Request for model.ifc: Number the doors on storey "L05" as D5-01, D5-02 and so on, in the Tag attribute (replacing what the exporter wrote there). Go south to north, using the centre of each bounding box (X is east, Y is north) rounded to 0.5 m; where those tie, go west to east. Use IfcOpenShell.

First a look at what the model holds.

```python
import ifcopenshell
import ifcopenshell.util.element
import ifcopenshell.util.placement

model = ifcopenshell.open("model.ifc")
print(model.schema)
storey = next(s for s in model.by_type("IfcBuildingStorey") if s.Name == "L05")
doors = [e for e in ifcopenshell.util.element.get_decomposition(storey) if e.is_a("IfcDoor")]
for e in sorted(doors, key=lambda e: e.id()):
    origin = ifcopenshell.util.placement.get_local_placement(e.ObjectPlacement)[:3, 3]
    print(e.id(), e.Tag, e.Name, origin.round(2) + 0.0, sep=" | ")
```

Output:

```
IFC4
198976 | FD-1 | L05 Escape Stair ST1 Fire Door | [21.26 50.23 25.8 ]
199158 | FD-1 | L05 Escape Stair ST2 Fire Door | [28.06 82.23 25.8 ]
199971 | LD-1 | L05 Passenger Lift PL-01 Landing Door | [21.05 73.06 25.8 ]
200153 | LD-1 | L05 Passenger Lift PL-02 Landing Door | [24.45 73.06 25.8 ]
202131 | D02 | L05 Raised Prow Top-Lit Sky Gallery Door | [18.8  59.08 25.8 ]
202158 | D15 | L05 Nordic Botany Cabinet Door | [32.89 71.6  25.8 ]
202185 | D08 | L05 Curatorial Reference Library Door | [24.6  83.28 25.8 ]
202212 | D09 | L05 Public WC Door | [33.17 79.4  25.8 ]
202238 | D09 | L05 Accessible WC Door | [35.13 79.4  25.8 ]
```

```python
import ifcopenshell
import ifcopenshell.geom
import ifcopenshell.util.element
import ifcopenshell.util.shape

model = ifcopenshell.open("model.ifc")
settings = ifcopenshell.geom.settings()
settings.set("use-world-coords", True)


def centre(element):
    shape = ifcopenshell.geom.create_shape(settings, element)
    return ifcopenshell.util.shape.get_bbox_centroid(shape.geometry)


storey = next(s for s in model.by_type("IfcBuildingStorey") if s.Name == "L05")
doors = [e for e in ifcopenshell.util.element.get_decomposition(storey) if e.is_a("IfcDoor")]

# Insertion points can sit at a corner or the storey origin, so sort by the geometry (in metres).
centres = {e: centre(e) for e in doors}
doors.sort(key=lambda e: (round(centres[e][1] / 0.5), centres[e][0]))

for i, e in enumerate(doors, start=1):
    number = f"D5-{i:02d}"
    e.Tag = number
    print(e.id(), number)

model.write("model_edited.ifc")
```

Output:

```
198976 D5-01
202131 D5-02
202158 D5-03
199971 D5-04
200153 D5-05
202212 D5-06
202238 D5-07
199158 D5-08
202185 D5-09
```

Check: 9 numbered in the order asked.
